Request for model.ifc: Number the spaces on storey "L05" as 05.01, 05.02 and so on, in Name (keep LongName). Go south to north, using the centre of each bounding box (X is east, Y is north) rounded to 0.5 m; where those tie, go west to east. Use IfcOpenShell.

First a look at what the model holds.

```python
import ifcopenshell
import ifcopenshell.util.element
import ifcopenshell.util.placement

model = ifcopenshell.open("model.ifc")
print(model.schema)
storey = next(s for s in model.by_type("IfcBuildingStorey") if s.Name == "L05")
spaces = [e for e in ifcopenshell.util.element.get_decomposition(storey) if e.is_a("IfcSpace")]
for e in sorted(spaces, key=lambda e: e.id()):
    origin = ifcopenshell.util.placement.get_local_placement(e.ObjectPlacement)[:3, 3]
    print(e.id(), e.Name, e.LongName, origin.round(2) + 0.0, sep=" | ")
```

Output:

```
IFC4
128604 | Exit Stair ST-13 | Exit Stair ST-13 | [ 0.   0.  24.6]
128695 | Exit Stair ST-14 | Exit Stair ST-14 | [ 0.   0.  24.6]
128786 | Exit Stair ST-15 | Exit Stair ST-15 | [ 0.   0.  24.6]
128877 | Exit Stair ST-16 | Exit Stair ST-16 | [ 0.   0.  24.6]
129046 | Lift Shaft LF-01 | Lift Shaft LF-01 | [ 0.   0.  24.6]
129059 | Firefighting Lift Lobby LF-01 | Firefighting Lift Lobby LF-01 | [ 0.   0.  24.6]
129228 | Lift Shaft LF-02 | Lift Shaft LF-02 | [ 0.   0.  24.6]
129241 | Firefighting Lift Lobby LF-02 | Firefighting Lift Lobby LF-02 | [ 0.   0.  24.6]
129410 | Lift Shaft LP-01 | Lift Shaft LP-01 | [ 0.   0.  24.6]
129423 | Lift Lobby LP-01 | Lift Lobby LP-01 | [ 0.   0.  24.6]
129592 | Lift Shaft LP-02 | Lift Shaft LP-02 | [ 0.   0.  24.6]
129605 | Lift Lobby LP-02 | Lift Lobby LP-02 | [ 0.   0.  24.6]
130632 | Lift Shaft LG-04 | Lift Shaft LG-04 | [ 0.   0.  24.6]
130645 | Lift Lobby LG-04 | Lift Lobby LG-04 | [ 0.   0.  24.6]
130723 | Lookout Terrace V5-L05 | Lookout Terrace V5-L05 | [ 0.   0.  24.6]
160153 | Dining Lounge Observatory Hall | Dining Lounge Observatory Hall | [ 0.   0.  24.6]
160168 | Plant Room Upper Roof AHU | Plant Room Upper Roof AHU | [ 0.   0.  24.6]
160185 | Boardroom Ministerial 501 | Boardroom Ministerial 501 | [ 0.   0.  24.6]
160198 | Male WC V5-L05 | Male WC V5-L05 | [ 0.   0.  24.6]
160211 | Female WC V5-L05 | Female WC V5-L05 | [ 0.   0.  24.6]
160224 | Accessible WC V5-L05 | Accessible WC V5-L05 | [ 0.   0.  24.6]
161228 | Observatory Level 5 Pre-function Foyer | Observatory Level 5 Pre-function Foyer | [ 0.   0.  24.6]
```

```python
import ifcopenshell
import ifcopenshell.geom
import ifcopenshell.util.element
import ifcopenshell.util.shape

model = ifcopenshell.open("model.ifc")
settings = ifcopenshell.geom.settings()
settings.set("use-world-coords", True)


def centre(element):
    shape = ifcopenshell.geom.create_shape(settings, element)
    return ifcopenshell.util.shape.get_bbox_centroid(shape.geometry)


storey = next(s for s in model.by_type("IfcBuildingStorey") if s.Name == "L05")
spaces = [e for e in ifcopenshell.util.element.get_decomposition(storey) if e.is_a("IfcSpace")]

# Insertion points can sit at a corner or the storey origin, so sort by the geometry (in metres).
centres = {e: centre(e) for e in spaces}
spaces.sort(key=lambda e: (round(centres[e][1] / 0.5), centres[e][0]))

for i, e in enumerate(spaces, start=1):
    number = f"05.{i:02d}"
    e.Name = number
    print(e.id(), number)

model.write("model-out.ifc")
```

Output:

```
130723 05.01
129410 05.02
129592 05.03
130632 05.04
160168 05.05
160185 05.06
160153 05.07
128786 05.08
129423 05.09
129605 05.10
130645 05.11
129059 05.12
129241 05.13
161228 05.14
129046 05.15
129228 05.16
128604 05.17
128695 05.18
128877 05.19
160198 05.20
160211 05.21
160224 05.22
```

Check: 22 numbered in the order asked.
